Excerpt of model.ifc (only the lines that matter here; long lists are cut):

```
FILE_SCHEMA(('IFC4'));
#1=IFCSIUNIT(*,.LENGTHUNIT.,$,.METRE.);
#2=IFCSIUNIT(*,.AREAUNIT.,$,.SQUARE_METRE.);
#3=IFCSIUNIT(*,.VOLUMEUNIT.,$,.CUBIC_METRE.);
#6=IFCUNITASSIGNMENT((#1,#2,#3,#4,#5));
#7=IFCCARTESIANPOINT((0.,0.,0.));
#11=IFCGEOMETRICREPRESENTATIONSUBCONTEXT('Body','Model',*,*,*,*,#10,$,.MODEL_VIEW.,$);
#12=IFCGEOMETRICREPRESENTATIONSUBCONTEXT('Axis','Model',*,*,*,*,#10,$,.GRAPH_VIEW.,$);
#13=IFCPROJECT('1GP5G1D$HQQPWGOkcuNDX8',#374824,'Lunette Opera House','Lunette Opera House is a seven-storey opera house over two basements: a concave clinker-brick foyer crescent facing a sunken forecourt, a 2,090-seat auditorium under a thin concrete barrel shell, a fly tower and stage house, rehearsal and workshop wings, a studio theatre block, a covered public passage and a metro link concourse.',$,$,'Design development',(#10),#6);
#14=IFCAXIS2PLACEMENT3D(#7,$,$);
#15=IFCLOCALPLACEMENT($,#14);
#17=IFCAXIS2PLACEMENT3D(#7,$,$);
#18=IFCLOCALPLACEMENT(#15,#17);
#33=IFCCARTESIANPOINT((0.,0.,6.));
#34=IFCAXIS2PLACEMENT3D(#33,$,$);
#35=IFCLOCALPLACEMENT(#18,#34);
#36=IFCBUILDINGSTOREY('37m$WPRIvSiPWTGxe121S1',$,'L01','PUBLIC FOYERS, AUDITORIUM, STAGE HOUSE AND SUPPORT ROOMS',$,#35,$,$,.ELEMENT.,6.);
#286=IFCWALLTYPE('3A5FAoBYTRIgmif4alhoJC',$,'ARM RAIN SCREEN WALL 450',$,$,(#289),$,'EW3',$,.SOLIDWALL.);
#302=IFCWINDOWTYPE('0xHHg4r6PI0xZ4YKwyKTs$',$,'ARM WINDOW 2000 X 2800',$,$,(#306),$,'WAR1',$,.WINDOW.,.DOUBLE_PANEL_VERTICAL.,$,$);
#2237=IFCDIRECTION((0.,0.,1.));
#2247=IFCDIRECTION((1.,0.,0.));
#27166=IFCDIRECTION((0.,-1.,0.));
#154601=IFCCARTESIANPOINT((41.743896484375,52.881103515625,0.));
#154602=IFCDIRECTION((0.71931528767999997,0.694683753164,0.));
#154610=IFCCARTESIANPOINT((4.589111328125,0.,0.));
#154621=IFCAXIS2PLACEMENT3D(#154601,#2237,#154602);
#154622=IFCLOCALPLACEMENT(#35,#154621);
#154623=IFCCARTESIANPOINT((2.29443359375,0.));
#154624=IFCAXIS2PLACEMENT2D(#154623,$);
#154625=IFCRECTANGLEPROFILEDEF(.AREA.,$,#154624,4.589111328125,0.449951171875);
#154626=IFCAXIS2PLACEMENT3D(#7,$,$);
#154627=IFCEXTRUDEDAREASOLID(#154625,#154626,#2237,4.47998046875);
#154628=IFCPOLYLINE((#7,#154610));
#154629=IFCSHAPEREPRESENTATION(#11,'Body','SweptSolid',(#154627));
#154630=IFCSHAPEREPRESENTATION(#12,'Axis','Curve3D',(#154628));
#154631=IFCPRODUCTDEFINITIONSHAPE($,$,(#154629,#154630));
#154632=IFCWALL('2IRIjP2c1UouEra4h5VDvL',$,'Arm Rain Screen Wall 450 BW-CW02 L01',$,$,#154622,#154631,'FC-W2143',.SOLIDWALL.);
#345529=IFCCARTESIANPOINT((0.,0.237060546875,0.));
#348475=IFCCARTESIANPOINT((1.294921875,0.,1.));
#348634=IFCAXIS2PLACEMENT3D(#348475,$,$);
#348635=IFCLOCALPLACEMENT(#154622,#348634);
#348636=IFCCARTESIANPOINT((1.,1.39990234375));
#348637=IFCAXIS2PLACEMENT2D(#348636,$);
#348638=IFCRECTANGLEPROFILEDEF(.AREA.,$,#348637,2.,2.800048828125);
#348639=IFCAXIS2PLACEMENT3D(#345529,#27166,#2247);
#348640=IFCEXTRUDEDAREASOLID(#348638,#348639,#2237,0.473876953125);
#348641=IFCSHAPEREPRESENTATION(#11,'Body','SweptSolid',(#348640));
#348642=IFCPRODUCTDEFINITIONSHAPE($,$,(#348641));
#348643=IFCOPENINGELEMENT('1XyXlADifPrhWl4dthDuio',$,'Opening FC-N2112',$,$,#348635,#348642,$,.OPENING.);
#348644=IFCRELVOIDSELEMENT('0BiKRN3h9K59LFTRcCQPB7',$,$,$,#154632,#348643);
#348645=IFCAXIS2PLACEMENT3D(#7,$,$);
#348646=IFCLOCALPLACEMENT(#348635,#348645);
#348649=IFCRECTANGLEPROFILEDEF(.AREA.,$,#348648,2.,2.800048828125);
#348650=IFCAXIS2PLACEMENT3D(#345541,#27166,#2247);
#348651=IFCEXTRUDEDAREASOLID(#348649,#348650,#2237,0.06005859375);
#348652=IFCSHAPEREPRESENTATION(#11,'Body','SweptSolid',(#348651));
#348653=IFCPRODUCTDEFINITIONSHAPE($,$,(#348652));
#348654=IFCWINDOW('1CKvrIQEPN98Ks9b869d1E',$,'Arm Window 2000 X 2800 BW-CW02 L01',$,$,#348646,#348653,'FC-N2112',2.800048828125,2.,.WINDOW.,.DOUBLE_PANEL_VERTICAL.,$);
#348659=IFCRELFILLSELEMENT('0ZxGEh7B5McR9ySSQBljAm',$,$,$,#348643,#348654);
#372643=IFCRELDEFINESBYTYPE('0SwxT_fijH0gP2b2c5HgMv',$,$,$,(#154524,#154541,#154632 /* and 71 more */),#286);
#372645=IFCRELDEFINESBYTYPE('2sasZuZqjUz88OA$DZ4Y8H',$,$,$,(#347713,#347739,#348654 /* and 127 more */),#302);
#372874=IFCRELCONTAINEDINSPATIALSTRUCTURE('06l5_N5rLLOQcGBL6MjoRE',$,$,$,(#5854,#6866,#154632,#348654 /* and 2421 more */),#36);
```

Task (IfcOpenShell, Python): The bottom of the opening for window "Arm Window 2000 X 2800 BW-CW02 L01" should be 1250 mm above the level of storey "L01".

```python
import numpy as np
import ifcopenshell
import ifcopenshell.api.geometry
import ifcopenshell.geom
import ifcopenshell.util.element
import ifcopenshell.util.placement
import ifcopenshell.util.shape
import ifcopenshell.util.unit

model = ifcopenshell.open("model.ifc")
unit_scale = ifcopenshell.util.unit.calculate_unit_scale(model)

window = model.by_guid("1CKvrIQEPN98Ks9b869d1E")
opening = window.FillsVoids[0].RelatingOpeningElement
storey = ifcopenshell.util.element.get_container(window, ifc_class="IfcBuildingStorey")
level = ifcopenshell.util.placement.get_local_placement(storey.ObjectPlacement)[2, 3]

# The opening's origin need not be at the sill, so measure its lowest point.
shape = ifcopenshell.geom.create_shape(ifcopenshell.geom.settings(), opening)
bottom = ifcopenshell.util.shape.get_shape_bottom_elevation(shape, shape.geometry) / unit_scale
dz = level + 1.25 / unit_scale - bottom

shift = np.array([0.0, 0.0, dz])
# The window is placed relative to its opening, so it follows when the opening moves.
matrix = ifcopenshell.util.placement.get_local_placement(opening.ObjectPlacement)
matrix[:3, 3] += shift
ifcopenshell.api.geometry.edit_object_placement(
    model, product=opening, matrix=matrix, is_si=False, should_transform_children=True
)

print(f"moved by {dz * unit_scale:+.3f} m")

model.write("model_updated.ifc")
```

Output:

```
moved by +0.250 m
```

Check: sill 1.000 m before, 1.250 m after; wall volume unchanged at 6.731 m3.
